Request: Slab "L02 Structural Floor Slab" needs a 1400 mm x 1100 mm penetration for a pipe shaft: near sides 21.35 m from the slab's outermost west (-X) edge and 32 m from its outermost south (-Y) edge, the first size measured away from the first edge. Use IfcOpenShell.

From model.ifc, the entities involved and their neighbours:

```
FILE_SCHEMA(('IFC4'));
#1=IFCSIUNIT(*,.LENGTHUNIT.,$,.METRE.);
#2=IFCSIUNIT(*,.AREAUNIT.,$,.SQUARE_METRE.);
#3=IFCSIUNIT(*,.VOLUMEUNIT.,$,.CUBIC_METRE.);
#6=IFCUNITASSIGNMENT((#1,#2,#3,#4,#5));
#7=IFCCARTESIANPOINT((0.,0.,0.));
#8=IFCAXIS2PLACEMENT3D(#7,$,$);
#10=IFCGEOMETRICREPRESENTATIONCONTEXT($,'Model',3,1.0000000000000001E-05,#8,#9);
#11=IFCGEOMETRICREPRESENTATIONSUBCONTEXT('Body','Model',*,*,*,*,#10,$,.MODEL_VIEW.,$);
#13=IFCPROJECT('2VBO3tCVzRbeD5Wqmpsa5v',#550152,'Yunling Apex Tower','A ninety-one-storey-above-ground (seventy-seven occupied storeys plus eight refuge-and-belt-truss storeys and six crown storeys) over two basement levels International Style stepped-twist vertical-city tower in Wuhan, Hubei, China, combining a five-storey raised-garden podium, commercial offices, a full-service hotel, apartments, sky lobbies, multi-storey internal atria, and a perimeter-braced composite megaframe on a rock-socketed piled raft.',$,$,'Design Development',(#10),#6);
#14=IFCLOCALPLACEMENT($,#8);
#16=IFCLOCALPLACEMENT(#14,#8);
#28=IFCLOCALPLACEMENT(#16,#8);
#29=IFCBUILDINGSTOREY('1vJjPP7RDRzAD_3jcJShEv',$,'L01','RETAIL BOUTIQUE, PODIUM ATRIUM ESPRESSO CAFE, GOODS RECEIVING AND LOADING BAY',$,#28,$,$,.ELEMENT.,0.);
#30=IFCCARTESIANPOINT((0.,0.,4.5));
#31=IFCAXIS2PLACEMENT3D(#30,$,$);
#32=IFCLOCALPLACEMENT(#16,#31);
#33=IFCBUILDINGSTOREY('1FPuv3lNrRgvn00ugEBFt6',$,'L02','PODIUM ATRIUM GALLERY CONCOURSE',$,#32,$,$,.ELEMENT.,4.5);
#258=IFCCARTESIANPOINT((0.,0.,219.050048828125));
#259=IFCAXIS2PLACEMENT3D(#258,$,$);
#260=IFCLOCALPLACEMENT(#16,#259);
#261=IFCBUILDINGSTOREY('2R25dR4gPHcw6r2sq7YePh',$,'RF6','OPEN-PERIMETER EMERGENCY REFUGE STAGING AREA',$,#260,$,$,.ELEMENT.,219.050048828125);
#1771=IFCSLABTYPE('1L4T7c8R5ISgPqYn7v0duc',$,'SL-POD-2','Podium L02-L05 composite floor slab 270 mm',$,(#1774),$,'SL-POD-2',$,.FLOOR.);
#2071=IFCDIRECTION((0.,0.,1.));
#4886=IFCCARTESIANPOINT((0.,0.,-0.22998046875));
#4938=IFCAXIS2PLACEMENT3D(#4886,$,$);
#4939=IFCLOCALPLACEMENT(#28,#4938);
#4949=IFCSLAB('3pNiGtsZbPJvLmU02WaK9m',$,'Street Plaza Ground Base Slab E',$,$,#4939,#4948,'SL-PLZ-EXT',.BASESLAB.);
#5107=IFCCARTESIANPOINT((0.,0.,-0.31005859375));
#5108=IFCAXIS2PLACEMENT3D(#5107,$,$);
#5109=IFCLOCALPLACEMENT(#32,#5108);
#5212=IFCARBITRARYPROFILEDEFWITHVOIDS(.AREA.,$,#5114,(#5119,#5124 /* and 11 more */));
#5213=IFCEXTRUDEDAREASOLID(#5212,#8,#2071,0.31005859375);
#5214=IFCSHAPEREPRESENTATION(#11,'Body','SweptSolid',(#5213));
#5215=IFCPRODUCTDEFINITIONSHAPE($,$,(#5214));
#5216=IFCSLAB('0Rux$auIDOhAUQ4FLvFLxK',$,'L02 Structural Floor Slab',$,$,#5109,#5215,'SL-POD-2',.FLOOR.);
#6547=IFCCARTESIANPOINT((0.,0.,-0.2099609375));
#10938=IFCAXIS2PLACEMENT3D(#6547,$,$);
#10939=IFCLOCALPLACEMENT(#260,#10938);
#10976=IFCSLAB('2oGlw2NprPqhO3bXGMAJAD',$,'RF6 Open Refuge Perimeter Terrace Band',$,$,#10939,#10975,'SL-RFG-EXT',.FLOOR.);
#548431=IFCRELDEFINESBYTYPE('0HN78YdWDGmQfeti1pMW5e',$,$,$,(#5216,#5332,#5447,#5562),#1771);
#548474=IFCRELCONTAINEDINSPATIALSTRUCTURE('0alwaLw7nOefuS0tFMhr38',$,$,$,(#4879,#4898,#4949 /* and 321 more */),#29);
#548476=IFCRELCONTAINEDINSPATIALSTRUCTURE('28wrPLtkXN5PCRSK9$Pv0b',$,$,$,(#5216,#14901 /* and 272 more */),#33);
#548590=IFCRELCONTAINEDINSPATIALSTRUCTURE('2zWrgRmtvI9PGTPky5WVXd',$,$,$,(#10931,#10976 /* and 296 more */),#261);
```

```python
import numpy as np
import ifcopenshell
import ifcopenshell.api.feature
import ifcopenshell.api.geometry
import ifcopenshell.api.root
import ifcopenshell.geom
import ifcopenshell.util.placement
import ifcopenshell.util.representation
import ifcopenshell.util.shape
import ifcopenshell.util.unit

model = ifcopenshell.open("model.ifc")
unit_scale = ifcopenshell.util.unit.calculate_unit_scale(model)
settings = ifcopenshell.geom.settings()


def volume(element):
    """Net volume in cubic metres, openings subtracted."""
    shape = ifcopenshell.geom.create_shape(settings, element)
    return ifcopenshell.util.shape.get_volume(shape.geometry)


slab = model.by_id(5216)
before = volume(slab)

# Extent in the slab's own axes, in metres. The edges named are its -X and -Y sides.
slab_shape = ifcopenshell.geom.create_shape(settings, slab)
vertices = ifcopenshell.util.shape.get_vertices(slab_shape.geometry)
x_min, y_min, bottom = vertices.min(axis=0)
top = vertices[:, 2].max()

opening = ifcopenshell.api.root.create_entity(model, ifc_class="IfcOpeningElement", name="Pipe shaft opening", predefined_type="OPENING")
context = ifcopenshell.util.representation.get_context(model, "Model", "Body", "MODEL_VIEW")
width, depth = 1.4, 1.1
outline = [(0.0, 0.0), (width, 0.0), (width, depth), (0.0, depth), (0.0, 0.0)]
# Overshoot both faces by 50 mm so the cut is clean.
shape = ifcopenshell.api.geometry.add_slab_representation(
    model, context=context, depth=top - bottom + 0.1, polyline=outline
)
ifcopenshell.api.geometry.assign_representation(model, product=opening, representation=shape)

matrix = ifcopenshell.util.placement.get_local_placement(slab.ObjectPlacement)
matrix[:, 3] = matrix @ np.append(np.array([x_min + 21.35, y_min + 32, bottom - 0.05]) / unit_scale, 1.0)
ifcopenshell.api.geometry.edit_object_placement(model, product=opening, matrix=matrix, is_si=False)
ifcopenshell.api.feature.add_feature(model, feature=opening, element=slab)

after = volume(slab)

print(f"slab volume {before:.3f} -> {after:.3f} m3")

model.write("model_edited.ifc")
```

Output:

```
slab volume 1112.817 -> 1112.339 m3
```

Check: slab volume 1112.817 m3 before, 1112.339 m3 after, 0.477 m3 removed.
